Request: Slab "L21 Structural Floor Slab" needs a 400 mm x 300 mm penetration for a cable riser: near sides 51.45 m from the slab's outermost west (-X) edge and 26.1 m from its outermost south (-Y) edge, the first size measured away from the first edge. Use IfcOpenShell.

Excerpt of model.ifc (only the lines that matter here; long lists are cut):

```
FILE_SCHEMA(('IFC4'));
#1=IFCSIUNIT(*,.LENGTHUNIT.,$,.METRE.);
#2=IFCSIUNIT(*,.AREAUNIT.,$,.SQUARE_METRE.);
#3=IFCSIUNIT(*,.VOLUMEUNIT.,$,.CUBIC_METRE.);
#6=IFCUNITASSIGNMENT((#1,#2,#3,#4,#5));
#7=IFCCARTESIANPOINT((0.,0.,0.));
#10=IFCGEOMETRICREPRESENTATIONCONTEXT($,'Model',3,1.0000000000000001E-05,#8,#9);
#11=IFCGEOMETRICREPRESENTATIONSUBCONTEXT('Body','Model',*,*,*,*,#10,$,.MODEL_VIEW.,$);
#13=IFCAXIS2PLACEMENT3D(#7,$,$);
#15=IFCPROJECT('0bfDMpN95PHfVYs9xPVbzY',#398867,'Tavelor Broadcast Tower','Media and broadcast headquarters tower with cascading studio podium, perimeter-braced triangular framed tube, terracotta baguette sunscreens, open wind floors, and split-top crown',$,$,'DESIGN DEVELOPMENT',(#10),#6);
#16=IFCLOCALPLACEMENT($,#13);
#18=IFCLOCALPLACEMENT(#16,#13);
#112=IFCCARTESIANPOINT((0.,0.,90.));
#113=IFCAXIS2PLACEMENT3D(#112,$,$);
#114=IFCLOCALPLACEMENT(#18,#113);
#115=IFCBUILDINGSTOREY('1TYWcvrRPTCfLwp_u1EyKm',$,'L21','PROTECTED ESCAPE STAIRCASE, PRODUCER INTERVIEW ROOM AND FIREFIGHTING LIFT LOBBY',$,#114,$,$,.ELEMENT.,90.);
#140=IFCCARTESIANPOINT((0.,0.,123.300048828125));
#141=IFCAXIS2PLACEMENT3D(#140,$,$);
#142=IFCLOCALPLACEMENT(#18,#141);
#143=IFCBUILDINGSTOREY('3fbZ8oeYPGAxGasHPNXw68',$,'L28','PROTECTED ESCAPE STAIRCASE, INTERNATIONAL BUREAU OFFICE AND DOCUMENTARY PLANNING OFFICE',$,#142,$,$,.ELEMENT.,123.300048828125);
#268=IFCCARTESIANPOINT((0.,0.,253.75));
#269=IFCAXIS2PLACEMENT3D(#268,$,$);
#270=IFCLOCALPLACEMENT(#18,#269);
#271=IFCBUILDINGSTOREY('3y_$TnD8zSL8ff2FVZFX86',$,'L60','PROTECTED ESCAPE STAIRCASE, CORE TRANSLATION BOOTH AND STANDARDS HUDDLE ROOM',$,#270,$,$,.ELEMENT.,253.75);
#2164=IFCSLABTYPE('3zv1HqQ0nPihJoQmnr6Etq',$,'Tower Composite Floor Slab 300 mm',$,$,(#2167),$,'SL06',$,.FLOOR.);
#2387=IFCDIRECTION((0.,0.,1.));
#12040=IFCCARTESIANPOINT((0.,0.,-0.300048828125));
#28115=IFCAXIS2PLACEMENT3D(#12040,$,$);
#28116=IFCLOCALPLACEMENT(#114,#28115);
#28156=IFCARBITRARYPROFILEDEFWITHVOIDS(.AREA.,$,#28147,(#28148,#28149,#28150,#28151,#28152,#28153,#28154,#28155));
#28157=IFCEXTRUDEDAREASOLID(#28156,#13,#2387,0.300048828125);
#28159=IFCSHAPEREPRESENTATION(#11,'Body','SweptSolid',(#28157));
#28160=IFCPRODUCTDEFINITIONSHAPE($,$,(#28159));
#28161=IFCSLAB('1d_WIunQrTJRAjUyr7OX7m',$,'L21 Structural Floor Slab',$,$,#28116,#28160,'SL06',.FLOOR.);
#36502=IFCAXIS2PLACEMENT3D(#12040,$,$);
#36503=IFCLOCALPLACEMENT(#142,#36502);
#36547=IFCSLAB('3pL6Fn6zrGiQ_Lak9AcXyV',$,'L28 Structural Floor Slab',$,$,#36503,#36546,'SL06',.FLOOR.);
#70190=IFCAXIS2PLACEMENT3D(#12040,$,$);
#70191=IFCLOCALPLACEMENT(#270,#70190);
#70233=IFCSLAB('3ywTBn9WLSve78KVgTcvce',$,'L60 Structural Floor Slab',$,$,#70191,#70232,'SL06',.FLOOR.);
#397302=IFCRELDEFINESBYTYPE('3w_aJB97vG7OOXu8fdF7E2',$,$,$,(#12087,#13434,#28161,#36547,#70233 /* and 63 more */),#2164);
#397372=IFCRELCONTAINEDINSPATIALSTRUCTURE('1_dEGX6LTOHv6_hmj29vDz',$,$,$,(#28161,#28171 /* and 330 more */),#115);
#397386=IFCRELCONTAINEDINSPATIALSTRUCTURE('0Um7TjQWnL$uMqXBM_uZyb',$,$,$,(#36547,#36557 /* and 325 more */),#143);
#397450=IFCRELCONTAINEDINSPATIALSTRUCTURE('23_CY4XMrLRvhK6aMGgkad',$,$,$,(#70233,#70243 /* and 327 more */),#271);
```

```python
import numpy as np
import ifcopenshell
import ifcopenshell.api.feature
import ifcopenshell.api.geometry
import ifcopenshell.api.root
import ifcopenshell.geom
import ifcopenshell.util.placement
import ifcopenshell.util.representation
import ifcopenshell.util.shape
import ifcopenshell.util.unit

model = ifcopenshell.open("model.ifc")
unit_scale = ifcopenshell.util.unit.calculate_unit_scale(model)
settings = ifcopenshell.geom.settings()


def volume(element):
    """Net volume in cubic metres, openings subtracted."""
    shape = ifcopenshell.geom.create_shape(settings, element)
    return ifcopenshell.util.shape.get_volume(shape.geometry)


slab = model.by_guid("1d_WIunQrTJRAjUyr7OX7m")
before = volume(slab)

# Extent in the slab's own axes, in metres. The edges named are its -X and -Y sides.
slab_shape = ifcopenshell.geom.create_shape(settings, slab)
vertices = ifcopenshell.util.shape.get_vertices(slab_shape.geometry)
x_min, y_min, bottom = vertices.min(axis=0)
top = vertices[:, 2].max()

opening = ifcopenshell.api.root.create_entity(model, ifc_class="IfcOpeningElement", name="Cable riser opening", predefined_type="OPENING")
context = ifcopenshell.util.representation.get_context(model, "Model", "Body", "MODEL_VIEW")
width, depth = 0.4, 0.3
outline = [(0.0, 0.0), (width, 0.0), (width, depth), (0.0, depth), (0.0, 0.0)]
# Overshoot both faces by 50 mm so the cut is clean.
shape = ifcopenshell.api.geometry.add_slab_representation(
    model, context=context, depth=top - bottom + 0.1, polyline=outline
)
ifcopenshell.api.geometry.assign_representation(model, product=opening, representation=shape)

matrix = ifcopenshell.util.placement.get_local_placement(slab.ObjectPlacement)
matrix[:, 3] = matrix @ np.append(np.array([x_min + 51.45, y_min + 26.1, bottom - 0.05]) / unit_scale, 1.0)
ifcopenshell.api.geometry.edit_object_placement(model, product=opening, matrix=matrix, is_si=False)
ifcopenshell.api.feature.add_feature(model, feature=opening, element=slab)

after = volume(slab)

print(f"slab volume {before:.3f} -> {after:.3f} m3")

model.write("model_updated.ifc")
```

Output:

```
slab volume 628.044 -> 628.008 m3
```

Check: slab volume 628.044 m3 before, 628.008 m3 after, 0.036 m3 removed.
